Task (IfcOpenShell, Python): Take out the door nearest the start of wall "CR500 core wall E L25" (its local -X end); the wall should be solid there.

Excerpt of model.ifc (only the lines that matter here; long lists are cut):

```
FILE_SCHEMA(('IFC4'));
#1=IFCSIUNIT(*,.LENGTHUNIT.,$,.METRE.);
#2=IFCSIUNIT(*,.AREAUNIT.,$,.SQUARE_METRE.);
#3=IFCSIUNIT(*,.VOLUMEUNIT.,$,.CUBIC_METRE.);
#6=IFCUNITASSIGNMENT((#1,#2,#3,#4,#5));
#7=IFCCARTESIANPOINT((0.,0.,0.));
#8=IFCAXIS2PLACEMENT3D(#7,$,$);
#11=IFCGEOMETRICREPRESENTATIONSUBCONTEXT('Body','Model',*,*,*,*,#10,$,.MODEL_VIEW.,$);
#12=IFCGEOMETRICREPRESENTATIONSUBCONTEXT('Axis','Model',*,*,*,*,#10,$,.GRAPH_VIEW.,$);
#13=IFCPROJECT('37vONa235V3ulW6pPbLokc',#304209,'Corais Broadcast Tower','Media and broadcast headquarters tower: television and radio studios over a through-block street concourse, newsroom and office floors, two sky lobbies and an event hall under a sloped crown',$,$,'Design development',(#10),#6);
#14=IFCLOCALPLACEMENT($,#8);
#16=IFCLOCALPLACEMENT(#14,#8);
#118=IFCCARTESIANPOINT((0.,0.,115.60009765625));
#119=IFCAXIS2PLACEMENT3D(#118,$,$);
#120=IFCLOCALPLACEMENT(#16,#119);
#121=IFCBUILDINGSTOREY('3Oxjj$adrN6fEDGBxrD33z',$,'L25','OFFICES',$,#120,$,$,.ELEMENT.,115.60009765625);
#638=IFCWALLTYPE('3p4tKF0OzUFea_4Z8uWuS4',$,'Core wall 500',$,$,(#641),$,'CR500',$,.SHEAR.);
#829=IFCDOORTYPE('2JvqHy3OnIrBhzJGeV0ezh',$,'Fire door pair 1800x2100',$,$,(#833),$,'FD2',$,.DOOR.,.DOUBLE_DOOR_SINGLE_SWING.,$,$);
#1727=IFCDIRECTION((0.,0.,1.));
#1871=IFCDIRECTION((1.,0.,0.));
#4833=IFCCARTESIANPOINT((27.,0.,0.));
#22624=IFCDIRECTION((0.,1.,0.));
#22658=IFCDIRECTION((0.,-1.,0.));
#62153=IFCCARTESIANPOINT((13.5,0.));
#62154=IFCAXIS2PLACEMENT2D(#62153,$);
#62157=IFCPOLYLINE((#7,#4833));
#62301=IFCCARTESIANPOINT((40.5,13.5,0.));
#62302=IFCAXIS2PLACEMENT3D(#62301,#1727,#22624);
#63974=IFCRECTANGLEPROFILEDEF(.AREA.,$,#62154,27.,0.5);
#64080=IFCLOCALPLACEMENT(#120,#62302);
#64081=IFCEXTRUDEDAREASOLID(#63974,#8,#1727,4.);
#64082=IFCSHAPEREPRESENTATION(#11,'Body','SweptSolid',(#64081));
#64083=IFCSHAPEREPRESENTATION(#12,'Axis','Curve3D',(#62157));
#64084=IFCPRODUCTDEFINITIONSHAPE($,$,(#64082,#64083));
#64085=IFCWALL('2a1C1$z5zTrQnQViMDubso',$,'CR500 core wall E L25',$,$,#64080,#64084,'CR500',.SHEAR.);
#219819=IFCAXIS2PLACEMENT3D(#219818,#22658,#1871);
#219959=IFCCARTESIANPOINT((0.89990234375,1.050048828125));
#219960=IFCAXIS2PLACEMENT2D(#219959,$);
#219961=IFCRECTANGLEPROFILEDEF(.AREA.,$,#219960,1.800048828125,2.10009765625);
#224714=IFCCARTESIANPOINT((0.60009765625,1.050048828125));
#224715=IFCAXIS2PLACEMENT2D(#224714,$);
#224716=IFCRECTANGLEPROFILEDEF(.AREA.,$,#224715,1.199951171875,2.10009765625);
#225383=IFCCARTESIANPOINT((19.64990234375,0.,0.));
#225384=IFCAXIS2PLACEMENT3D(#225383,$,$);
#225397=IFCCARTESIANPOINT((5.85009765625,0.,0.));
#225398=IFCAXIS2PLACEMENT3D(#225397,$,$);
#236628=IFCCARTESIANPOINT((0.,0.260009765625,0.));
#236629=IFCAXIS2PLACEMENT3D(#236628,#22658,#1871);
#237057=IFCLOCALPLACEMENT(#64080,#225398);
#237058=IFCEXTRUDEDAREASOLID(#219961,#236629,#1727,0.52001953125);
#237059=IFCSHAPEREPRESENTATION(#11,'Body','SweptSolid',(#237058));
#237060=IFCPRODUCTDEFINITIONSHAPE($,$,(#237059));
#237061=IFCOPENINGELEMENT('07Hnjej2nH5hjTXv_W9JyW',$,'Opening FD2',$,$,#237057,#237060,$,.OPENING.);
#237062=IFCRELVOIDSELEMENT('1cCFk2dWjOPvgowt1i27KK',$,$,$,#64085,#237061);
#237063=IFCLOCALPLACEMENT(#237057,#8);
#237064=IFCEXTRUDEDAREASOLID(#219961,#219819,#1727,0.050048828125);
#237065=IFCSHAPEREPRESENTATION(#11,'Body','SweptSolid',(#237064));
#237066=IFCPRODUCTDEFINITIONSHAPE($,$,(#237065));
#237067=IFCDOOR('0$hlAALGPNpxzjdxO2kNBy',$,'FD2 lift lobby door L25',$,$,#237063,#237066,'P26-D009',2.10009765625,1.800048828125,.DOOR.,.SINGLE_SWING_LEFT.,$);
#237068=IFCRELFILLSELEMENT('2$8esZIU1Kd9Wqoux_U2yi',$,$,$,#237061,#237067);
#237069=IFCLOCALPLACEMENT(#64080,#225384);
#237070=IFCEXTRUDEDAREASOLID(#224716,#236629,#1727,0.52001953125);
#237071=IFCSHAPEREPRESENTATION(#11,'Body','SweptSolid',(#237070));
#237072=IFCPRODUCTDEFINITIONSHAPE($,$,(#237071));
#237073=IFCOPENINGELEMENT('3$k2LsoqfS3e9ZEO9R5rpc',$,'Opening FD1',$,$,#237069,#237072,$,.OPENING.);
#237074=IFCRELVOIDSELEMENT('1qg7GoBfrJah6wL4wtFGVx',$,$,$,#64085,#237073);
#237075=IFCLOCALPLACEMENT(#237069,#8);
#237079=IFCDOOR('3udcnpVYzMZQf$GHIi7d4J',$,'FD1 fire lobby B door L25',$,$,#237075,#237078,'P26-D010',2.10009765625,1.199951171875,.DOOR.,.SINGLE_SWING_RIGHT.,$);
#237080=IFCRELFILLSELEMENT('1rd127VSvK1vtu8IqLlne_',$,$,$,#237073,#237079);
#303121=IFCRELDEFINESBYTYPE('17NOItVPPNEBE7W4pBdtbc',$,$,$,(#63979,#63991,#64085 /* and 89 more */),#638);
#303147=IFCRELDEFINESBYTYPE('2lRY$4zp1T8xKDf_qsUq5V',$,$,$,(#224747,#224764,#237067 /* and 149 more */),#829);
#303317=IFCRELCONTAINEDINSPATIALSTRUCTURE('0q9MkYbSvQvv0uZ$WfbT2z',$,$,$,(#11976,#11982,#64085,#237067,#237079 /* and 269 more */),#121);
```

```python
import ifcopenshell
import ifcopenshell.api.feature
import ifcopenshell.api.root
import ifcopenshell.geom
import ifcopenshell.util.shape

model = ifcopenshell.open("model.ifc")
settings = ifcopenshell.geom.settings()


def volume(element):
    """Net volume in cubic metres, openings subtracted."""
    shape = ifcopenshell.geom.create_shape(settings, element)
    return ifcopenshell.util.shape.get_volume(shape.geometry)


door = model.by_guid("0$hlAALGPNpxzjdxO2kNBy")
opening = door.FillsVoids[0].RelatingOpeningElement
wall = opening.VoidsElements[0].RelatingBuildingElement
before = volume(wall)

ifcopenshell.api.root.remove_product(model, product=door)
ifcopenshell.api.feature.remove_feature(model, feature=opening)

after = volume(wall)

print(f"wall volume {before:.3f} -> {after:.3f} m3")

model.write("model_v2.ifc")
```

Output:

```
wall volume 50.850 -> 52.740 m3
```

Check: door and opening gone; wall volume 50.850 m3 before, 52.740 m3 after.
